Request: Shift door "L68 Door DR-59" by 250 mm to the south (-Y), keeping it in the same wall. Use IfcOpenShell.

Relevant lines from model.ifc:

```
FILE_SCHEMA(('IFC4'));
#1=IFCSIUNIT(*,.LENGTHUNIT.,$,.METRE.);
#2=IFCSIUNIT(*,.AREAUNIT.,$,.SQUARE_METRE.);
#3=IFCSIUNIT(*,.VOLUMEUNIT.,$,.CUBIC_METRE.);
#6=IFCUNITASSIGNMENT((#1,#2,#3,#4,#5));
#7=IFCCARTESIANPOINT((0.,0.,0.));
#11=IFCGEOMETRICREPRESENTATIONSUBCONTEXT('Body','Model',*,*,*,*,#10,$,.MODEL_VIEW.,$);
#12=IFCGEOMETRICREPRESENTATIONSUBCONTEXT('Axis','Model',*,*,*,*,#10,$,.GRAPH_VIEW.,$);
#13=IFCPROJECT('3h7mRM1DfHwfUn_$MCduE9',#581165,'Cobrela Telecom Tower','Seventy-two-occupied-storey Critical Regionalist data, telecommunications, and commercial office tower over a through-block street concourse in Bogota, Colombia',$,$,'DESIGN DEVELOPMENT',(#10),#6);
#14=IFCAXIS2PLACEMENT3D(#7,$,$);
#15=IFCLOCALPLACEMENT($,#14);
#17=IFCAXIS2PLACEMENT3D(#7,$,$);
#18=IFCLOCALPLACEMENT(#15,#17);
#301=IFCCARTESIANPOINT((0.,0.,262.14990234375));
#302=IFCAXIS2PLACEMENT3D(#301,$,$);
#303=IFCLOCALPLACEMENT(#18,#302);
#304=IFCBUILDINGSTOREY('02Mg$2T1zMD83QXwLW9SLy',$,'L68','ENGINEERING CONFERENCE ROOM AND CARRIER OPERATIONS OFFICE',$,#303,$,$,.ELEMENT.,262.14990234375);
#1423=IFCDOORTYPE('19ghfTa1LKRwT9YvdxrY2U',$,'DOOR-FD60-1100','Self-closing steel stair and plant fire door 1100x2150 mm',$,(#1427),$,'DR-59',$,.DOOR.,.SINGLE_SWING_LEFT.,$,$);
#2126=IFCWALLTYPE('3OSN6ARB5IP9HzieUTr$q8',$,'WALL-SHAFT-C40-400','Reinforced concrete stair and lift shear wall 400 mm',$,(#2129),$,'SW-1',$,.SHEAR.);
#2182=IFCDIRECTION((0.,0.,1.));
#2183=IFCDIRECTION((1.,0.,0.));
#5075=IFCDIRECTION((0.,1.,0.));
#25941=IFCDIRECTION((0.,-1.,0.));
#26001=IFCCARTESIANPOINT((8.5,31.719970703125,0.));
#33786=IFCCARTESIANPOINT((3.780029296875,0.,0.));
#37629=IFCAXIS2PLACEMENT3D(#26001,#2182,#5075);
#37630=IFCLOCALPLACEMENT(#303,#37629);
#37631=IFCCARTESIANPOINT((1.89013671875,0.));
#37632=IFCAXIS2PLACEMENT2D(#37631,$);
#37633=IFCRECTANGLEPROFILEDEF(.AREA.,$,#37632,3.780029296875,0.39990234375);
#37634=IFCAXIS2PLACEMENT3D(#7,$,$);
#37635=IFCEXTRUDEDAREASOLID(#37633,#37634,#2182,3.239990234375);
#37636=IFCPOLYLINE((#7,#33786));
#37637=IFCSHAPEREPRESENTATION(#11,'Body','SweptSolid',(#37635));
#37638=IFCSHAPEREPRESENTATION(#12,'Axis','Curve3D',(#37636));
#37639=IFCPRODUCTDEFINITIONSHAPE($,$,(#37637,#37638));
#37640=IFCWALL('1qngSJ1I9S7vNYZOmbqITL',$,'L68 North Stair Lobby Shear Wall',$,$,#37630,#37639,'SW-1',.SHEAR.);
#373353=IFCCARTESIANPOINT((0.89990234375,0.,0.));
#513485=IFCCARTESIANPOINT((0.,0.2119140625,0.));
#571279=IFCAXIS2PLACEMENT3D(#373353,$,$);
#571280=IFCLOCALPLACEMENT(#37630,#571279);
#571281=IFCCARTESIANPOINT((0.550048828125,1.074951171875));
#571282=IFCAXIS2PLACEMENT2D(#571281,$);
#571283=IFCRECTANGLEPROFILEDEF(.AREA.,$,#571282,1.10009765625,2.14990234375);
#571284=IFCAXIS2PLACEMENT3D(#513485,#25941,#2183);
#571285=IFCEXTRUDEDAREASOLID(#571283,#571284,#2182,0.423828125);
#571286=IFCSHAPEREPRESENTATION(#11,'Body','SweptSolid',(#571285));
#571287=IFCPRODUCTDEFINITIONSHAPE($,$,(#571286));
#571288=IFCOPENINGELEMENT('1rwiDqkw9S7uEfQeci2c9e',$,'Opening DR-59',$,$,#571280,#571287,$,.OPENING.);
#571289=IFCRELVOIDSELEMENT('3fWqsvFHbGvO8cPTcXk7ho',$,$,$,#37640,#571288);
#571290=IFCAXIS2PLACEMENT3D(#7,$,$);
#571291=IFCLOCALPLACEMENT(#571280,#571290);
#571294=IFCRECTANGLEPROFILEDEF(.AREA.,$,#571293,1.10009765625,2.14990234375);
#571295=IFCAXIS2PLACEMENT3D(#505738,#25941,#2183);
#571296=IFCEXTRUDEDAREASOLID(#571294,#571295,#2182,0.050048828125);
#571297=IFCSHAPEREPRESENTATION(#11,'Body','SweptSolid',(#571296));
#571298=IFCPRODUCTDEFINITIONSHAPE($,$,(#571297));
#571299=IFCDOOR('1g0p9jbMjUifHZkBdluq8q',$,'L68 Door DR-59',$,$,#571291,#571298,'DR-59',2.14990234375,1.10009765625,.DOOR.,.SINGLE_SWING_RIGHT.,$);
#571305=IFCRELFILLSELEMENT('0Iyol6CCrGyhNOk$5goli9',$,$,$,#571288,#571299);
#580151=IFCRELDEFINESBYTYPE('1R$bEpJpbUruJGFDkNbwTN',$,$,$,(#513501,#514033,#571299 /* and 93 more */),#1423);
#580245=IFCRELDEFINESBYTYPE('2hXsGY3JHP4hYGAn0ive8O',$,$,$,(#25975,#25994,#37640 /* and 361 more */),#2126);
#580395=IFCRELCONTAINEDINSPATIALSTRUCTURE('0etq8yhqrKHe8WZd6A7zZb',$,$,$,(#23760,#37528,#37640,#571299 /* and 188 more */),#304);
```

```python
import ifcopenshell
import ifcopenshell.api.geometry
import ifcopenshell.util.placement
import ifcopenshell.util.unit

model = ifcopenshell.open("model.ifc")
unit_scale = ifcopenshell.util.unit.calculate_unit_scale(model)

door = model.by_id(571299)
opening = door.FillsVoids[0].RelatingOpeningElement
wall = opening.VoidsElements[0].RelatingBuildingElement

wall_matrix = ifcopenshell.util.placement.get_local_placement(wall.ObjectPlacement)
shift = wall_matrix[:3, 0] * -0.25 / unit_scale
before = ifcopenshell.util.placement.get_local_placement(door.ObjectPlacement)[:3, 3].copy()

# The door is placed relative to its opening, so it follows when the opening moves.
matrix = ifcopenshell.util.placement.get_local_placement(opening.ObjectPlacement)
matrix[:3, 3] += shift
ifcopenshell.api.geometry.edit_object_placement(
    model, product=opening, matrix=matrix, is_si=False, should_transform_children=True
)

after = ifcopenshell.util.placement.get_local_placement(door.ObjectPlacement)[:3, 3]
print("door moved by", (after - before).round(3) + 0.0)

model.write("model_updated.ifc")
```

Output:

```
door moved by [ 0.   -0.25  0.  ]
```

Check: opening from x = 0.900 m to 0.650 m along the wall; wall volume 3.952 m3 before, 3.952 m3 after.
